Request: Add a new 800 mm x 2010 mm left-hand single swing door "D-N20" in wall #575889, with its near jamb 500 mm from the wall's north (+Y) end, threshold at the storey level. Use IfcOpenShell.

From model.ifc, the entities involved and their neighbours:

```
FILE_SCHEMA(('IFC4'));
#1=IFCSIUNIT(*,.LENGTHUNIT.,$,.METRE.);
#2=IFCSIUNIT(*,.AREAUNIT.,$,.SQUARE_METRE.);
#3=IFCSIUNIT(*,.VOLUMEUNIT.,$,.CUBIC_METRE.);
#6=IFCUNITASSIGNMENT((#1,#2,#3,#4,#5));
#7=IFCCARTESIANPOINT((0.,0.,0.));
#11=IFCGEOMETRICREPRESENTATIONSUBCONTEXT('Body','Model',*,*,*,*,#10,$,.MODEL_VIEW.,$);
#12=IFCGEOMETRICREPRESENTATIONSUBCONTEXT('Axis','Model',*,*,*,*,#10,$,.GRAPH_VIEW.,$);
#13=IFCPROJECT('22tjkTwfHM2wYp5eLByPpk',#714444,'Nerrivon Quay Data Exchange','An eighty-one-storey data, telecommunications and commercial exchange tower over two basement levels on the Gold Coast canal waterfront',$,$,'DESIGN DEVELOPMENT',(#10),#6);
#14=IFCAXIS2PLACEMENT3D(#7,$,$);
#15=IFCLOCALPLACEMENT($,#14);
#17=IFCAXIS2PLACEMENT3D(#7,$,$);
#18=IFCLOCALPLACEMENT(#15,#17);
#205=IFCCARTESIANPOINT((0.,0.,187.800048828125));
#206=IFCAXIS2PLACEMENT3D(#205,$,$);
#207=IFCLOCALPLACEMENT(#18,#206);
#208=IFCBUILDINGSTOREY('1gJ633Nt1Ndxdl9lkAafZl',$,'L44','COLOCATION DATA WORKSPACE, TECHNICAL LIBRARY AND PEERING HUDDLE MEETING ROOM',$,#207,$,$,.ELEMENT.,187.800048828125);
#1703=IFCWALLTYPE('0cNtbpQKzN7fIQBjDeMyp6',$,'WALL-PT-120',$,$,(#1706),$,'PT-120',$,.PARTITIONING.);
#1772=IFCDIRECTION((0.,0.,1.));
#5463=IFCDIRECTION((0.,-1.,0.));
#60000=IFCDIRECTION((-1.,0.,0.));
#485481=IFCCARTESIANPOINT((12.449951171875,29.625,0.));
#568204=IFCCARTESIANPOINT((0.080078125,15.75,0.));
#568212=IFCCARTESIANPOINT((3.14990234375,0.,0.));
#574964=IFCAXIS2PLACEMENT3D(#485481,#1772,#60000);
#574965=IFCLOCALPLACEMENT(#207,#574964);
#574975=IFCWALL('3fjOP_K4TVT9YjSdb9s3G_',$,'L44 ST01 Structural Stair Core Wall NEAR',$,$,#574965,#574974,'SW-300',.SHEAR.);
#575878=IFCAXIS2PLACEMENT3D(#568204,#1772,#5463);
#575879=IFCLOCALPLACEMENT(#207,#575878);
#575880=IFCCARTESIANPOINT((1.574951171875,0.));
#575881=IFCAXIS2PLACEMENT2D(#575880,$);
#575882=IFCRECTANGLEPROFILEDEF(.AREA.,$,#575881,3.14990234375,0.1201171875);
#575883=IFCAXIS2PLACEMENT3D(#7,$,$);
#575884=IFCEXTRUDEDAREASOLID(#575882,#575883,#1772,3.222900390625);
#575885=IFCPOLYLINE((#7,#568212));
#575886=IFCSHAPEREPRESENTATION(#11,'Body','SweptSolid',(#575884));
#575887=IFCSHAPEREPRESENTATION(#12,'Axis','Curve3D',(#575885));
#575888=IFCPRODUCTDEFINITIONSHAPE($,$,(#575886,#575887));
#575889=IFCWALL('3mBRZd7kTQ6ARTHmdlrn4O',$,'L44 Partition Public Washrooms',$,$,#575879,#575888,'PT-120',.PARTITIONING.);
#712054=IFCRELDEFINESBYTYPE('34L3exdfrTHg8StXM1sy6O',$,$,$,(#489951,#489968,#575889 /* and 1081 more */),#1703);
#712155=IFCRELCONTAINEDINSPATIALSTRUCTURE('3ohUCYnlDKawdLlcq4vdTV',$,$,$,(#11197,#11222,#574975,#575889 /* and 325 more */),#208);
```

```python
import numpy as np
import ifcopenshell
import ifcopenshell.api.feature
import ifcopenshell.api.geometry
import ifcopenshell.api.root
import ifcopenshell.api.spatial
import ifcopenshell.geom
import ifcopenshell.util.element
import ifcopenshell.util.placement
import ifcopenshell.util.representation
import ifcopenshell.util.shape
import ifcopenshell.util.unit

model = ifcopenshell.open("model.ifc")
unit_scale = ifcopenshell.util.unit.calculate_unit_scale(model)
settings = ifcopenshell.geom.settings()


def volume(element):
    """Net volume in cubic metres, openings subtracted."""
    shape = ifcopenshell.geom.create_shape(settings, element)
    return ifcopenshell.util.shape.get_volume(shape.geometry)


wall = model.by_guid("3mBRZd7kTQ6ARTHmdlrn4O")
storey = ifcopenshell.util.element.get_container(wall, ifc_class="IfcBuildingStorey")
context = ifcopenshell.util.representation.get_context(model, "Model", "Body", "MODEL_VIEW")
before = volume(wall)

width, height, from_end, sill = 0.8, 2.01, 0.5, 0.0  # metres

# The wall runs along its own X axis, and the end named is its -X end.
wall_shape = ifcopenshell.geom.create_shape(settings, wall)
x, y, z = ifcopenshell.util.shape.get_vertices(wall_shape.geometry).T
start = x.min() + from_end
face, thickness = float(y.min()), float(y.max() - y.min())
wall_matrix = ifcopenshell.util.placement.get_local_placement(wall.ObjectPlacement)
level = ifcopenshell.util.placement.get_local_placement(storey.ObjectPlacement)[2, 3]


def in_wall(x, y):
    """Placement at x, y metres in the wall's axes, at sill height."""
    matrix = wall_matrix.copy()
    matrix[:, 3] = wall_matrix @ np.array([x / unit_scale, y / unit_scale, 0.0, 1.0])
    matrix[2, 3] = level + sill / unit_scale
    return matrix


# Opening: a box that overshoots both wall faces by 50 mm.
opening = ifcopenshell.api.root.create_entity(model, ifc_class="IfcOpeningElement", predefined_type="OPENING")
box = ifcopenshell.api.geometry.add_wall_representation(
    model, context=context, length=width, height=height, thickness=thickness + 0.1
)
ifcopenshell.api.geometry.assign_representation(model, product=opening, representation=box)
ifcopenshell.api.geometry.edit_object_placement(model, product=opening, matrix=in_wall(start, face - 0.05), is_si=False)
ifcopenshell.api.feature.add_feature(model, feature=opening, element=wall)

door = ifcopenshell.api.root.create_entity(model, ifc_class="IfcDoor", name="D-N20", predefined_type="DOOR")
door.OverallWidth, door.OverallHeight = width / unit_scale, height / unit_scale
door.OperationType = "SINGLE_SWING_LEFT"
body = ifcopenshell.api.geometry.add_door_representation(
    model,
    context=context,
    overall_width=door.OverallWidth,
    overall_height=door.OverallHeight,
    operation_type="SINGLE_SWING_LEFT",
    lining_properties={"LiningDepth": thickness / unit_scale, "ThresholdDepth": thickness / unit_scale},
)
ifcopenshell.api.geometry.assign_representation(model, product=door, representation=body)
ifcopenshell.api.spatial.assign_container(model, products=[door], relating_structure=storey)
ifcopenshell.api.feature.add_filling(model, opening=opening, element=door)

# The lining spans the wall, so the door starts at the wall face.
ifcopenshell.api.geometry.edit_object_placement(model, product=door, matrix=in_wall(start, face), is_si=False)

after = volume(wall)

print(f"wall volume {before:.3f} -> {after:.3f} m3")

model.write("model_edited.ifc")
```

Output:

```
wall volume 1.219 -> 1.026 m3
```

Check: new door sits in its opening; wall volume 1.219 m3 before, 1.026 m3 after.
